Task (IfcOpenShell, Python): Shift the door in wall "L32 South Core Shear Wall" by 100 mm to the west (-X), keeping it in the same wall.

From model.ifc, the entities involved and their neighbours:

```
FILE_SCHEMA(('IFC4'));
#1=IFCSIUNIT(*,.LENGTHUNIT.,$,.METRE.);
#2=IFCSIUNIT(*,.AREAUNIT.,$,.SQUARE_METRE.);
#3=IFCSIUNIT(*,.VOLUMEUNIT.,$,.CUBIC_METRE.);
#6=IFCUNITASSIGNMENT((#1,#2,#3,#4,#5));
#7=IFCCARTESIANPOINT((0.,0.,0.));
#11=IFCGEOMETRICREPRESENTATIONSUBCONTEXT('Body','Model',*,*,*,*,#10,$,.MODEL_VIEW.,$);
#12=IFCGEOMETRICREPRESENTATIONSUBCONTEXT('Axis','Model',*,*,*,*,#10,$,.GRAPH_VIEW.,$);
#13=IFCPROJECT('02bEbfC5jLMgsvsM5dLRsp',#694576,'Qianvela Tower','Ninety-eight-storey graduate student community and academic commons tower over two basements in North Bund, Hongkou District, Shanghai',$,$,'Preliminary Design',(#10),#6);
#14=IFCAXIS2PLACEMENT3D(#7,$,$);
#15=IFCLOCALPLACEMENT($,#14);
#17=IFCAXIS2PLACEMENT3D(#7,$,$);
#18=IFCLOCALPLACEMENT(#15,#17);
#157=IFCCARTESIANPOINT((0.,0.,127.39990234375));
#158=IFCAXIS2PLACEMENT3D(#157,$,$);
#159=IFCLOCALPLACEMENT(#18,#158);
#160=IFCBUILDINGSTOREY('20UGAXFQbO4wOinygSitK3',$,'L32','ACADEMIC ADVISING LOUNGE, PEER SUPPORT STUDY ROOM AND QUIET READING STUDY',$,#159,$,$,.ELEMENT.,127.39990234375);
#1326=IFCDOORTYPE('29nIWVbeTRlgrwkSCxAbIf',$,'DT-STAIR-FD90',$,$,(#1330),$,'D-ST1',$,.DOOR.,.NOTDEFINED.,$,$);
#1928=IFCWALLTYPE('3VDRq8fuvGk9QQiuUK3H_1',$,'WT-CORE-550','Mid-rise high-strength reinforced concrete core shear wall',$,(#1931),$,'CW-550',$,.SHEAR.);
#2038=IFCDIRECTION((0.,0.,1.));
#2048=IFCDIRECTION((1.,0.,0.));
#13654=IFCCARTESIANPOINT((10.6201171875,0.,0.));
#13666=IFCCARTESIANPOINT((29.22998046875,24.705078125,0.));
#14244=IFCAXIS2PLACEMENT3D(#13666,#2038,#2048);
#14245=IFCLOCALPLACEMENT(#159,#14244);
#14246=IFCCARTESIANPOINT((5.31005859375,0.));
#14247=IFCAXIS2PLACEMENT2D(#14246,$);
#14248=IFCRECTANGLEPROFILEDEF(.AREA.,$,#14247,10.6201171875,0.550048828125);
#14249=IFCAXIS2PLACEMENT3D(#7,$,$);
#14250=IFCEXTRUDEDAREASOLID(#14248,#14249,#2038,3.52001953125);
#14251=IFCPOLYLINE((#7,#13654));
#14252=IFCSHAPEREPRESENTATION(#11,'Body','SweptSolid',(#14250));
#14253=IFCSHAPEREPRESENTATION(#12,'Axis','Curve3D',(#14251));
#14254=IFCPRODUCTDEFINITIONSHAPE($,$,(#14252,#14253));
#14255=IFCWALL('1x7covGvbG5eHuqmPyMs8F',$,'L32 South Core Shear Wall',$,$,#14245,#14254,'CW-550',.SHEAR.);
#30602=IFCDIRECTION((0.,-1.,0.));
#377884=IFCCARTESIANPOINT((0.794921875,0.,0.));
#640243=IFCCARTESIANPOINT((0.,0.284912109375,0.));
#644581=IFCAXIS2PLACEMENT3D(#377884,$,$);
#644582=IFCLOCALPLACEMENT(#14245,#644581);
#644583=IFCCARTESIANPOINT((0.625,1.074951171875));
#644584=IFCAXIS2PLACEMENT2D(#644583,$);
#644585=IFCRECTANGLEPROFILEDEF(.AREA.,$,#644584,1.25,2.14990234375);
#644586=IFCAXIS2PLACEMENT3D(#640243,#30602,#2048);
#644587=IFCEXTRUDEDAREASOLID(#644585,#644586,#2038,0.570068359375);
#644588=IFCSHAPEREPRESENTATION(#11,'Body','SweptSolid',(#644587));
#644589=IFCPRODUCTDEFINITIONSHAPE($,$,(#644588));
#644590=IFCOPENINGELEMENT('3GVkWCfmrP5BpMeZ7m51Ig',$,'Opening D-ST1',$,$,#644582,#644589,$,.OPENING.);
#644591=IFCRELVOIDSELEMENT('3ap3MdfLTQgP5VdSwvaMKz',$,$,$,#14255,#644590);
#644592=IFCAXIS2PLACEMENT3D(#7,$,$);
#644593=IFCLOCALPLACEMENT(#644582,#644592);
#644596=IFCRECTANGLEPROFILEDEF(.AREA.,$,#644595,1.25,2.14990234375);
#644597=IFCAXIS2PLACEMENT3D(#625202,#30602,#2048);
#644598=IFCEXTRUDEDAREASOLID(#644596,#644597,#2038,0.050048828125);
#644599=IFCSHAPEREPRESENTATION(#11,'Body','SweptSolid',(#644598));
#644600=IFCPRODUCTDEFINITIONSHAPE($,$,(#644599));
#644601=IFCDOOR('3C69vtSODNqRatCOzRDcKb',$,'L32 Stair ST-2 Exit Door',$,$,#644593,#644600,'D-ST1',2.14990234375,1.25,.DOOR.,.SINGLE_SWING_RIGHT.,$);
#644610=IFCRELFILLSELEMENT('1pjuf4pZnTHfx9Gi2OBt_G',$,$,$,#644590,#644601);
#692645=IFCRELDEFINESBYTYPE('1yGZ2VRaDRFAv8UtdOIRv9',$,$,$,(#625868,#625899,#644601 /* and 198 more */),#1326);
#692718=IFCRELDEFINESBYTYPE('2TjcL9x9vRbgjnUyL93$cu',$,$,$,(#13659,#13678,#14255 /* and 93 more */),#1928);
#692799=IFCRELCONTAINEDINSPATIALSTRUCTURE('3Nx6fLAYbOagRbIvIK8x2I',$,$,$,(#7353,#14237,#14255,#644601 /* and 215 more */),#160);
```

```python
import ifcopenshell
import ifcopenshell.api.geometry
import ifcopenshell.util.placement
import ifcopenshell.util.unit

model = ifcopenshell.open("model.ifc")
unit_scale = ifcopenshell.util.unit.calculate_unit_scale(model)

door = model.by_guid("3C69vtSODNqRatCOzRDcKb")
opening = door.FillsVoids[0].RelatingOpeningElement
wall = opening.VoidsElements[0].RelatingBuildingElement

wall_matrix = ifcopenshell.util.placement.get_local_placement(wall.ObjectPlacement)
shift = wall_matrix[:3, 0] * -0.1 / unit_scale
before = ifcopenshell.util.placement.get_local_placement(door.ObjectPlacement)[:3, 3].copy()

# The door is placed relative to its opening, so it follows when the opening moves.
matrix = ifcopenshell.util.placement.get_local_placement(opening.ObjectPlacement)
matrix[:3, 3] += shift
ifcopenshell.api.geometry.edit_object_placement(
    model, product=opening, matrix=matrix, is_si=False, should_transform_children=True
)

after = ifcopenshell.util.placement.get_local_placement(door.ObjectPlacement)[:3, 3]
print("door moved by", (after - before).round(3) + 0.0)

model.write("model_rev.ifc")
```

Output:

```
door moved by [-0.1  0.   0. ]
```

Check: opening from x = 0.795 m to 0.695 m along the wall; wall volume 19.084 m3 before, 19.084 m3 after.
